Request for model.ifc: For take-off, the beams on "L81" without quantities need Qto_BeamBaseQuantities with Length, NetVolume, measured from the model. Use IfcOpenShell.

First a look at what the model holds.

```python
import ifcopenshell
import ifcopenshell.util.element
import ifcopenshell.util.unit

model = ifcopenshell.open("model.ifc")
print(model.schema)
for unit_type in ("LENGTHUNIT", "AREAUNIT", "VOLUMEUNIT"):
    print(unit_type, ifcopenshell.util.unit.calculate_unit_scale(model, unit_type))
storey = next(s for s in model.by_type("IfcBuildingStorey") if s.Name == "L81")
beams = [e for e in ifcopenshell.util.element.get_decomposition(storey) if e.is_a("IfcBeam")]
for e in sorted(beams, key=lambda e: e.id()):
    print(e.id(), e.is_a(), e.Name, list(ifcopenshell.util.element.get_psets(e, qtos_only=True)), sep=" | ")
```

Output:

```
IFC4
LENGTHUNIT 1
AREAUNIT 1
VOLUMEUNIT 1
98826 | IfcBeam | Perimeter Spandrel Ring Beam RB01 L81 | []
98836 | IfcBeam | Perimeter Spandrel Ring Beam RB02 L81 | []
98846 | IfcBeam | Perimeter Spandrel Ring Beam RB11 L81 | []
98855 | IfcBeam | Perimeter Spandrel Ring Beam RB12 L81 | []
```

```python
import ifcopenshell
import ifcopenshell.api.pset
import ifcopenshell.geom
import ifcopenshell.util.element
import ifcopenshell.util.shape
import ifcopenshell.util.unit

model = ifcopenshell.open("model.ifc")
unit_scale = ifcopenshell.util.unit.calculate_unit_scale(model)
volume_scale = ifcopenshell.util.unit.calculate_unit_scale(model, "VOLUMEUNIT")
settings = ifcopenshell.geom.settings()

storey = next(s for s in model.by_type("IfcBuildingStorey") if s.Name == "L81")
beams = [e for e in ifcopenshell.util.element.get_decomposition(storey) if e.is_a("IfcBeam")]

for e in sorted(beams, key=lambda e: e.id()):
    if ifcopenshell.util.element.get_psets(e, qtos_only=True, should_inherit=False):
        continue
    # Geometry comes back in metres, in the element's own axes.
    shape = ifcopenshell.geom.create_shape(settings, e)
    values = {
        "Length": ifcopenshell.util.shape.get_max_xyz(shape.geometry) / unit_scale,
        "NetVolume": ifcopenshell.util.shape.get_volume(shape.geometry) / volume_scale,
    }
    qto = ifcopenshell.api.pset.add_qto(model, product=e, name="Qto_BeamBaseQuantities")
    ifcopenshell.api.pset.edit_qto(model, qto=qto, properties=values)
    print(e.id(), {k: round(v, 3) for k, v in values.items()})

model.write("model_rev.ifc")
```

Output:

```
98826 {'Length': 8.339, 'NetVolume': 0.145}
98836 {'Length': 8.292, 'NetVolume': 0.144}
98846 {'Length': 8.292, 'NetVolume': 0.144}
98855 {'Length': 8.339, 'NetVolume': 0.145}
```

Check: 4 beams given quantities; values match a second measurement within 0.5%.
